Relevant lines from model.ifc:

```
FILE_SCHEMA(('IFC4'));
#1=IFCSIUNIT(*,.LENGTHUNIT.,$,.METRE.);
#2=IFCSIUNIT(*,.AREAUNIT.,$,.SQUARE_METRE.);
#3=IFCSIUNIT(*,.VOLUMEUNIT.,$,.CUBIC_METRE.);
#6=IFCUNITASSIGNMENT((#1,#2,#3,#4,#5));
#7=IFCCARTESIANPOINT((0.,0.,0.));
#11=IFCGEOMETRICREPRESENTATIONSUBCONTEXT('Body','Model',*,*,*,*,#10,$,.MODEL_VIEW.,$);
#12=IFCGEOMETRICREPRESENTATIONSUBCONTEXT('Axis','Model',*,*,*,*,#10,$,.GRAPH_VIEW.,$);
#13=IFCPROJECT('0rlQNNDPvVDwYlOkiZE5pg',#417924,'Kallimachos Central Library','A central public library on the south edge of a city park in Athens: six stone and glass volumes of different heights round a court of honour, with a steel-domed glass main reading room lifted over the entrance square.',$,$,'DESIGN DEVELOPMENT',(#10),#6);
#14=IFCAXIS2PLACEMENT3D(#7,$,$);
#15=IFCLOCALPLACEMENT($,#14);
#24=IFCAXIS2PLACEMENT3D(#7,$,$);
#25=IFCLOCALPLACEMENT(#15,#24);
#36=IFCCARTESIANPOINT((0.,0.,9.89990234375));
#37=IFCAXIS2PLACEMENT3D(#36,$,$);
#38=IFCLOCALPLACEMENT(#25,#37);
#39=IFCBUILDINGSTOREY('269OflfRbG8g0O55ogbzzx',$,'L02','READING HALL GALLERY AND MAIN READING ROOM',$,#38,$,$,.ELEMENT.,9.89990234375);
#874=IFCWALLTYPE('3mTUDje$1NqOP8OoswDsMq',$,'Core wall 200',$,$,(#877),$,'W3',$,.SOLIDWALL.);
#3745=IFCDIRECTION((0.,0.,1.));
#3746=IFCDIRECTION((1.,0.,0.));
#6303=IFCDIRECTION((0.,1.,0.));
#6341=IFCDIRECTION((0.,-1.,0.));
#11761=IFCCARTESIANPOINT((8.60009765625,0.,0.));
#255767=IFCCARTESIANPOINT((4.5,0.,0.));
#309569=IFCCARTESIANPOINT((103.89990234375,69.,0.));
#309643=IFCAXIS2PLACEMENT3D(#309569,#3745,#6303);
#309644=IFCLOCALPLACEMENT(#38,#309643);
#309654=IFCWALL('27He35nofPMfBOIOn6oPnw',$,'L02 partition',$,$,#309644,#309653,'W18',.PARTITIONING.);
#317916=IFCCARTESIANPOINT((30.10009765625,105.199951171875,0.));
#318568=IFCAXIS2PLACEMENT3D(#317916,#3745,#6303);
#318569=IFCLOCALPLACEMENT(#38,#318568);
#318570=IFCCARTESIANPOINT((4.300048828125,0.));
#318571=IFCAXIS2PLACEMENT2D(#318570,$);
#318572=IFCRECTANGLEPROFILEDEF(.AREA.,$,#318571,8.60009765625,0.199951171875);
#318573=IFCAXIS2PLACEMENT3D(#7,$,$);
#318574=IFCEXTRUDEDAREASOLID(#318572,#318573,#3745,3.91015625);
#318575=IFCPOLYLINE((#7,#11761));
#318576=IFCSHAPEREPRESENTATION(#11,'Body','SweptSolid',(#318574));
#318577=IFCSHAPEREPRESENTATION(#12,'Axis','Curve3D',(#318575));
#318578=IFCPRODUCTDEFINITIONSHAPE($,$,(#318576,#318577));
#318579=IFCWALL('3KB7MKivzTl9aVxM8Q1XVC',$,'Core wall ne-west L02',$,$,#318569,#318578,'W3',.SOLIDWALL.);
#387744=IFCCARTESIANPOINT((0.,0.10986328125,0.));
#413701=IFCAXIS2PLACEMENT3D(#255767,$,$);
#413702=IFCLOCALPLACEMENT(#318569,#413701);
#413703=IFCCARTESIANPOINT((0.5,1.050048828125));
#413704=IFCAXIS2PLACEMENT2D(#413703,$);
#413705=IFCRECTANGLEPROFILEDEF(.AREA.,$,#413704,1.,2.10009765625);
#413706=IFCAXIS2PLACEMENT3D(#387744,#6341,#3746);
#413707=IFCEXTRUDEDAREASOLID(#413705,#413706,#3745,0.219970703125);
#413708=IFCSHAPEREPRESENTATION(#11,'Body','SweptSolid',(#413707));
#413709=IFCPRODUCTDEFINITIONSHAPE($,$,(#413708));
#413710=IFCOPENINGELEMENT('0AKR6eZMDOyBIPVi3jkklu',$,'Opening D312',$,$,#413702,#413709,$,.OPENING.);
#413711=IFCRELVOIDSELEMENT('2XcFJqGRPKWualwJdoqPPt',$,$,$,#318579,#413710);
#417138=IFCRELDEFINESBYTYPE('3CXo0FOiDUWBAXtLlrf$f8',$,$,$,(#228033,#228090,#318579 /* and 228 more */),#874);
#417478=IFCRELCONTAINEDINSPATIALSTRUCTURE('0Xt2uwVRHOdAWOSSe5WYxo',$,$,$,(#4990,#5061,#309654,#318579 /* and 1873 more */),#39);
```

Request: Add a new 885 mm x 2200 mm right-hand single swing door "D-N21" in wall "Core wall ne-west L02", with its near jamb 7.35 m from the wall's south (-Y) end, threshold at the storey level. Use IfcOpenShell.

```python
import numpy as np
import ifcopenshell
import ifcopenshell.api.feature
import ifcopenshell.api.geometry
import ifcopenshell.api.root
import ifcopenshell.api.spatial
import ifcopenshell.geom
import ifcopenshell.util.element
import ifcopenshell.util.placement
import ifcopenshell.util.representation
import ifcopenshell.util.shape
import ifcopenshell.util.unit

model = ifcopenshell.open("model.ifc")
unit_scale = ifcopenshell.util.unit.calculate_unit_scale(model)
settings = ifcopenshell.geom.settings()


def volume(element):
    """Net volume in cubic metres, openings subtracted."""
    shape = ifcopenshell.geom.create_shape(settings, element)
    return ifcopenshell.util.shape.get_volume(shape.geometry)


wall = model.by_id(318579)
storey = ifcopenshell.util.element.get_container(wall, ifc_class="IfcBuildingStorey")
context = ifcopenshell.util.representation.get_context(model, "Model", "Body", "MODEL_VIEW")
before = volume(wall)

width, height, from_end, sill = 0.885, 2.2, 7.35, 0.0  # metres

# The wall runs along its own X axis, and the end named is its -X end.
wall_shape = ifcopenshell.geom.create_shape(settings, wall)
x, y, z = ifcopenshell.util.shape.get_vertices(wall_shape.geometry).T
start = x.min() + from_end
face, thickness = float(y.min()), float(y.max() - y.min())
wall_matrix = ifcopenshell.util.placement.get_local_placement(wall.ObjectPlacement)
level = ifcopenshell.util.placement.get_local_placement(storey.ObjectPlacement)[2, 3]


def in_wall(x, y):
    """Placement at x, y metres in the wall's axes, at sill height."""
    matrix = wall_matrix.copy()
    matrix[:, 3] = wall_matrix @ np.array([x / unit_scale, y / unit_scale, 0.0, 1.0])
    matrix[2, 3] = level + sill / unit_scale
    return matrix


# Opening: a box that overshoots both wall faces by 50 mm.
opening = ifcopenshell.api.root.create_entity(model, ifc_class="IfcOpeningElement", predefined_type="OPENING")
box = ifcopenshell.api.geometry.add_wall_representation(
    model, context=context, length=width, height=height, thickness=thickness + 0.1
)
ifcopenshell.api.geometry.assign_representation(model, product=opening, representation=box)
ifcopenshell.api.geometry.edit_object_placement(model, product=opening, matrix=in_wall(start, face - 0.05), is_si=False)
ifcopenshell.api.feature.add_feature(model, feature=opening, element=wall)

door = ifcopenshell.api.root.create_entity(model, ifc_class="IfcDoor", name="D-N21", predefined_type="DOOR")
door.OverallWidth, door.OverallHeight = width / unit_scale, height / unit_scale
door.OperationType = "SINGLE_SWING_RIGHT"
body = ifcopenshell.api.geometry.add_door_representation(
    model,
    context=context,
    overall_width=door.OverallWidth,
    overall_height=door.OverallHeight,
    operation_type="SINGLE_SWING_RIGHT",
    lining_properties={"LiningDepth": thickness / unit_scale, "ThresholdDepth": thickness / unit_scale},
)
ifcopenshell.api.geometry.assign_representation(model, product=door, representation=body)
ifcopenshell.api.spatial.assign_container(model, products=[door], relating_structure=storey)
ifcopenshell.api.feature.add_filling(model, opening=opening, element=door)

# The lining spans the wall, so the door starts at the wall face.
ifcopenshell.api.geometry.edit_object_placement(model, product=door, matrix=in_wall(start, face), is_si=False)

after = volume(wall)

print(f"wall volume {before:.3f} -> {after:.3f} m3")

model.write("model_updated.ifc")
```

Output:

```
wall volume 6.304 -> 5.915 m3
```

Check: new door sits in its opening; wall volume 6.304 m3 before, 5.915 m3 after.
